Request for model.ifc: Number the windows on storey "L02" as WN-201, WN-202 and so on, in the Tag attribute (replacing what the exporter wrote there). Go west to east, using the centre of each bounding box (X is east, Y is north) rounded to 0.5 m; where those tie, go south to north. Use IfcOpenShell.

First a look at what the model holds.

```python
import ifcopenshell
import ifcopenshell.util.element
import ifcopenshell.util.placement

model = ifcopenshell.open("model.ifc")
print(model.schema)
storey = next(s for s in model.by_type("IfcBuildingStorey") if s.Name == "L02")
windows = [e for e in ifcopenshell.util.element.get_decomposition(storey) if e.is_a("IfcWindow")]
for e in sorted(windows, key=lambda e: e.id()):
    origin = ifcopenshell.util.placement.get_local_placement(e.ObjectPlacement)[:3, 3]
    print(e.id(), e.Tag, e.Name, origin.round(2) + 0.0, sep=" | ")
```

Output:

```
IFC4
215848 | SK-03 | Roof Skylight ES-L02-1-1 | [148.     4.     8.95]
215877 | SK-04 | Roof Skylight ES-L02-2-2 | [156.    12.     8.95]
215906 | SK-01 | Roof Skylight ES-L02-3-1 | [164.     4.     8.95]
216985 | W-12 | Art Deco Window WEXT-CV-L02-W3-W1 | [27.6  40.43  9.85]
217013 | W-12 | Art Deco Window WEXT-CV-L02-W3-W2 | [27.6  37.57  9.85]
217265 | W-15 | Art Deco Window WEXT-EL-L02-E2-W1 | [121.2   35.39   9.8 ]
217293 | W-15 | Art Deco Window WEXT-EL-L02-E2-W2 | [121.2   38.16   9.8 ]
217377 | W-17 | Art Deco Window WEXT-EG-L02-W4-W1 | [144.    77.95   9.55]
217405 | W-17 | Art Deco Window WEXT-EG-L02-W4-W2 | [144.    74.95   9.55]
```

```python
import ifcopenshell
import ifcopenshell.geom
import ifcopenshell.util.element
import ifcopenshell.util.shape

model = ifcopenshell.open("model.ifc")
settings = ifcopenshell.geom.settings()
settings.set("use-world-coords", True)


def centre(element):
    shape = ifcopenshell.geom.create_shape(settings, element)
    return ifcopenshell.util.shape.get_bbox_centroid(shape.geometry)


storey = next(s for s in model.by_type("IfcBuildingStorey") if s.Name == "L02")
windows = [e for e in ifcopenshell.util.element.get_decomposition(storey) if e.is_a("IfcWindow")]

# Insertion points can sit at a corner or the storey origin, so sort by the geometry (in metres).
centres = {e: centre(e) for e in windows}
windows.sort(key=lambda e: (round(centres[e][0] / 0.5), centres[e][1]))

for i, e in enumerate(windows, start=1):
    number = f"WN-2{i:02d}"
    e.Tag = number
    print(e.id(), number)

model.write("model_updated.ifc")
```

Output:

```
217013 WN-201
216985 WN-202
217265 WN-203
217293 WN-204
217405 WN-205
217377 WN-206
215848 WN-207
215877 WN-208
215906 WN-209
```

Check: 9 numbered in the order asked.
